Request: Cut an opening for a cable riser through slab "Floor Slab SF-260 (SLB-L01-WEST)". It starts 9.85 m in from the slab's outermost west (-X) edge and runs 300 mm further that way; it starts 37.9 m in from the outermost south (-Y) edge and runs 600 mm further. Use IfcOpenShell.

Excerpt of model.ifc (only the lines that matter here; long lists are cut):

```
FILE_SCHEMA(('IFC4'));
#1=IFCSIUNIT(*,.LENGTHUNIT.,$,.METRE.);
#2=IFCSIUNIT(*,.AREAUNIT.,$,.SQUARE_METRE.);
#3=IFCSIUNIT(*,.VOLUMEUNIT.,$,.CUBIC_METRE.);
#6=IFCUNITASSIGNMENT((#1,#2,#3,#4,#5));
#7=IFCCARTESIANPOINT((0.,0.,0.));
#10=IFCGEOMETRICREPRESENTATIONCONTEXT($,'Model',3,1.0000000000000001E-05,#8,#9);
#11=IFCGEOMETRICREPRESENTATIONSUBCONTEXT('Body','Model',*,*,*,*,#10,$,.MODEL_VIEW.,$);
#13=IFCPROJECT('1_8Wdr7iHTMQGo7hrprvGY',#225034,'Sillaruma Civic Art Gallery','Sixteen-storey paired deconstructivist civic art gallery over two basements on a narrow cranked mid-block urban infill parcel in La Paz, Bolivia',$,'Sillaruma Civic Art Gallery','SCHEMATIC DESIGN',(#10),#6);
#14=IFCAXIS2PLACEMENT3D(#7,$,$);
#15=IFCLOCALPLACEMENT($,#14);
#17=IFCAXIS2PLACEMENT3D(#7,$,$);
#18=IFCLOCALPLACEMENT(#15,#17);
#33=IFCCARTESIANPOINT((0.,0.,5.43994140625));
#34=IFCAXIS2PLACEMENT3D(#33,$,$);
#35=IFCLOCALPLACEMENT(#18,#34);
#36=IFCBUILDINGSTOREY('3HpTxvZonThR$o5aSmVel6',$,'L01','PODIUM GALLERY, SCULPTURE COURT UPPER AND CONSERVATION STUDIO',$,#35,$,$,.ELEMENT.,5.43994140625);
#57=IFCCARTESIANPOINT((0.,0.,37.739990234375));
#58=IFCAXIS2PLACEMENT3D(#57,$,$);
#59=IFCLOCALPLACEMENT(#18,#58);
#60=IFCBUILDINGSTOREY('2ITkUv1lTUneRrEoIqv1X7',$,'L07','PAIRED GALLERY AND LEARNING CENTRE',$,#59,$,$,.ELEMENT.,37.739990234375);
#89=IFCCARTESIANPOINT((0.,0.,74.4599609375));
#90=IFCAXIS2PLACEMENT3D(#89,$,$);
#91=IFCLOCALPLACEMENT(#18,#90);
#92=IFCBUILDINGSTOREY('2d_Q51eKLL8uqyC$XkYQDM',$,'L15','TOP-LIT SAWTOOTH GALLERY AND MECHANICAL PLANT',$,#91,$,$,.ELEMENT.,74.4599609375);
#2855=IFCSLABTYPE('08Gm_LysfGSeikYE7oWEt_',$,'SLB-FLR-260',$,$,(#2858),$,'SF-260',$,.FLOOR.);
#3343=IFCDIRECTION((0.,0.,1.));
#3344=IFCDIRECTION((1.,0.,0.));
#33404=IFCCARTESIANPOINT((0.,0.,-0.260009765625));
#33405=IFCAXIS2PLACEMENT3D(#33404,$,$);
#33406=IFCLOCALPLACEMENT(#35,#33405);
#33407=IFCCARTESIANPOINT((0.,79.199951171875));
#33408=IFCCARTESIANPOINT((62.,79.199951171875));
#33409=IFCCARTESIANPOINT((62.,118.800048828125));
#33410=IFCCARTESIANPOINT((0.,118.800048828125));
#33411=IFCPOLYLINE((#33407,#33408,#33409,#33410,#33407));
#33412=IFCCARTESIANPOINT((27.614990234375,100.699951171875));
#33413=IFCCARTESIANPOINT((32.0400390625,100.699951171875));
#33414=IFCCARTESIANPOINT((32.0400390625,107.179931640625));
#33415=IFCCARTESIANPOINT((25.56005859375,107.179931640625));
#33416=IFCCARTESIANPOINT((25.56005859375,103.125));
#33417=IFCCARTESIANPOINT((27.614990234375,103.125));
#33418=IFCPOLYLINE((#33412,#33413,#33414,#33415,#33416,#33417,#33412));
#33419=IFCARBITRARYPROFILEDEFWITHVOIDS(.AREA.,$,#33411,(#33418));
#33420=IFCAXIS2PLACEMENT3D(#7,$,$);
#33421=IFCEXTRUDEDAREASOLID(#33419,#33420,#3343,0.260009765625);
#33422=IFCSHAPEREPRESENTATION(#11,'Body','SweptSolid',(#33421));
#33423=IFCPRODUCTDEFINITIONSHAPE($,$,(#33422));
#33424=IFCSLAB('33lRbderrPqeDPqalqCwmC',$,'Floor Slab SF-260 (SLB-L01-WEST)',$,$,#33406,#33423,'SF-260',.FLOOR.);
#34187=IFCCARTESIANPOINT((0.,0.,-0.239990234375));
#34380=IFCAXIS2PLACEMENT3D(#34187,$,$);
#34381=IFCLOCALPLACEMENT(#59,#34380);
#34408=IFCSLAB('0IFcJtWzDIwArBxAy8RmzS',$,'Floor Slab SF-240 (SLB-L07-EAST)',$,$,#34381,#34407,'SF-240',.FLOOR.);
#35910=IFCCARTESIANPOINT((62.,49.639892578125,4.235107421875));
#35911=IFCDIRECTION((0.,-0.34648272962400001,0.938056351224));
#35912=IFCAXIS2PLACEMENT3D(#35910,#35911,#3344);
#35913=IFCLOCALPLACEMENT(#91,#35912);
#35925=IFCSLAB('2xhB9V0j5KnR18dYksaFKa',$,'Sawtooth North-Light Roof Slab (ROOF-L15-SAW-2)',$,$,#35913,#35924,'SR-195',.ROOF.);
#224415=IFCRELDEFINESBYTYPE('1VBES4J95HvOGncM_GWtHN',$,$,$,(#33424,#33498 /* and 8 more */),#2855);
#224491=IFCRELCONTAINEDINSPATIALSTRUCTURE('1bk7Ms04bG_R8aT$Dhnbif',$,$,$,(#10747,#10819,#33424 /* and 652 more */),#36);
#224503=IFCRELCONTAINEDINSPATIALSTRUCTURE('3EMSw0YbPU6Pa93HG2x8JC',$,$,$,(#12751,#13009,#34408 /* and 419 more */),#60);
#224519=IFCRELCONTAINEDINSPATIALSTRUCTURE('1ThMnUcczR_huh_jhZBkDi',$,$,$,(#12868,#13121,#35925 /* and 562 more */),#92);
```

```python
import numpy as np
import ifcopenshell
import ifcopenshell.api.feature
import ifcopenshell.api.geometry
import ifcopenshell.api.root
import ifcopenshell.geom
import ifcopenshell.util.placement
import ifcopenshell.util.representation
import ifcopenshell.util.shape
import ifcopenshell.util.unit

model = ifcopenshell.open("model.ifc")
unit_scale = ifcopenshell.util.unit.calculate_unit_scale(model)
settings = ifcopenshell.geom.settings()


def volume(element):
    """Net volume in cubic metres, openings subtracted."""
    shape = ifcopenshell.geom.create_shape(settings, element)
    return ifcopenshell.util.shape.get_volume(shape.geometry)


slab = model.by_guid("33lRbderrPqeDPqalqCwmC")
before = volume(slab)

# Extent in the slab's own axes, in metres. The edges named are its -X and -Y sides.
slab_shape = ifcopenshell.geom.create_shape(settings, slab)
vertices = ifcopenshell.util.shape.get_vertices(slab_shape.geometry)
x_min, y_min, bottom = vertices.min(axis=0)
top = vertices[:, 2].max()

opening = ifcopenshell.api.root.create_entity(model, ifc_class="IfcOpeningElement", name="Cable riser opening", predefined_type="OPENING")
context = ifcopenshell.util.representation.get_context(model, "Model", "Body", "MODEL_VIEW")
width, depth = 0.3, 0.6
outline = [(0.0, 0.0), (width, 0.0), (width, depth), (0.0, depth), (0.0, 0.0)]
# Overshoot both faces by 50 mm so the cut is clean.
shape = ifcopenshell.api.geometry.add_slab_representation(
    model, context=context, depth=top - bottom + 0.1, polyline=outline
)
ifcopenshell.api.geometry.assign_representation(model, product=opening, representation=shape)

matrix = ifcopenshell.util.placement.get_local_placement(slab.ObjectPlacement)
matrix[:, 3] = matrix @ np.append(np.array([x_min + 9.85, y_min + 37.9, bottom - 0.05]) / unit_scale, 1.0)
ifcopenshell.api.geometry.edit_object_placement(model, product=opening, matrix=matrix, is_si=False)
ifcopenshell.api.feature.add_feature(model, feature=opening, element=slab)

after = volume(slab)

print(f"slab volume {before:.3f} -> {after:.3f} m3")

model.write("model_v2.ifc")
```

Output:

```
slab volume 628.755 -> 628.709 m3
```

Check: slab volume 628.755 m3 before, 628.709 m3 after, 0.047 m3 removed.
